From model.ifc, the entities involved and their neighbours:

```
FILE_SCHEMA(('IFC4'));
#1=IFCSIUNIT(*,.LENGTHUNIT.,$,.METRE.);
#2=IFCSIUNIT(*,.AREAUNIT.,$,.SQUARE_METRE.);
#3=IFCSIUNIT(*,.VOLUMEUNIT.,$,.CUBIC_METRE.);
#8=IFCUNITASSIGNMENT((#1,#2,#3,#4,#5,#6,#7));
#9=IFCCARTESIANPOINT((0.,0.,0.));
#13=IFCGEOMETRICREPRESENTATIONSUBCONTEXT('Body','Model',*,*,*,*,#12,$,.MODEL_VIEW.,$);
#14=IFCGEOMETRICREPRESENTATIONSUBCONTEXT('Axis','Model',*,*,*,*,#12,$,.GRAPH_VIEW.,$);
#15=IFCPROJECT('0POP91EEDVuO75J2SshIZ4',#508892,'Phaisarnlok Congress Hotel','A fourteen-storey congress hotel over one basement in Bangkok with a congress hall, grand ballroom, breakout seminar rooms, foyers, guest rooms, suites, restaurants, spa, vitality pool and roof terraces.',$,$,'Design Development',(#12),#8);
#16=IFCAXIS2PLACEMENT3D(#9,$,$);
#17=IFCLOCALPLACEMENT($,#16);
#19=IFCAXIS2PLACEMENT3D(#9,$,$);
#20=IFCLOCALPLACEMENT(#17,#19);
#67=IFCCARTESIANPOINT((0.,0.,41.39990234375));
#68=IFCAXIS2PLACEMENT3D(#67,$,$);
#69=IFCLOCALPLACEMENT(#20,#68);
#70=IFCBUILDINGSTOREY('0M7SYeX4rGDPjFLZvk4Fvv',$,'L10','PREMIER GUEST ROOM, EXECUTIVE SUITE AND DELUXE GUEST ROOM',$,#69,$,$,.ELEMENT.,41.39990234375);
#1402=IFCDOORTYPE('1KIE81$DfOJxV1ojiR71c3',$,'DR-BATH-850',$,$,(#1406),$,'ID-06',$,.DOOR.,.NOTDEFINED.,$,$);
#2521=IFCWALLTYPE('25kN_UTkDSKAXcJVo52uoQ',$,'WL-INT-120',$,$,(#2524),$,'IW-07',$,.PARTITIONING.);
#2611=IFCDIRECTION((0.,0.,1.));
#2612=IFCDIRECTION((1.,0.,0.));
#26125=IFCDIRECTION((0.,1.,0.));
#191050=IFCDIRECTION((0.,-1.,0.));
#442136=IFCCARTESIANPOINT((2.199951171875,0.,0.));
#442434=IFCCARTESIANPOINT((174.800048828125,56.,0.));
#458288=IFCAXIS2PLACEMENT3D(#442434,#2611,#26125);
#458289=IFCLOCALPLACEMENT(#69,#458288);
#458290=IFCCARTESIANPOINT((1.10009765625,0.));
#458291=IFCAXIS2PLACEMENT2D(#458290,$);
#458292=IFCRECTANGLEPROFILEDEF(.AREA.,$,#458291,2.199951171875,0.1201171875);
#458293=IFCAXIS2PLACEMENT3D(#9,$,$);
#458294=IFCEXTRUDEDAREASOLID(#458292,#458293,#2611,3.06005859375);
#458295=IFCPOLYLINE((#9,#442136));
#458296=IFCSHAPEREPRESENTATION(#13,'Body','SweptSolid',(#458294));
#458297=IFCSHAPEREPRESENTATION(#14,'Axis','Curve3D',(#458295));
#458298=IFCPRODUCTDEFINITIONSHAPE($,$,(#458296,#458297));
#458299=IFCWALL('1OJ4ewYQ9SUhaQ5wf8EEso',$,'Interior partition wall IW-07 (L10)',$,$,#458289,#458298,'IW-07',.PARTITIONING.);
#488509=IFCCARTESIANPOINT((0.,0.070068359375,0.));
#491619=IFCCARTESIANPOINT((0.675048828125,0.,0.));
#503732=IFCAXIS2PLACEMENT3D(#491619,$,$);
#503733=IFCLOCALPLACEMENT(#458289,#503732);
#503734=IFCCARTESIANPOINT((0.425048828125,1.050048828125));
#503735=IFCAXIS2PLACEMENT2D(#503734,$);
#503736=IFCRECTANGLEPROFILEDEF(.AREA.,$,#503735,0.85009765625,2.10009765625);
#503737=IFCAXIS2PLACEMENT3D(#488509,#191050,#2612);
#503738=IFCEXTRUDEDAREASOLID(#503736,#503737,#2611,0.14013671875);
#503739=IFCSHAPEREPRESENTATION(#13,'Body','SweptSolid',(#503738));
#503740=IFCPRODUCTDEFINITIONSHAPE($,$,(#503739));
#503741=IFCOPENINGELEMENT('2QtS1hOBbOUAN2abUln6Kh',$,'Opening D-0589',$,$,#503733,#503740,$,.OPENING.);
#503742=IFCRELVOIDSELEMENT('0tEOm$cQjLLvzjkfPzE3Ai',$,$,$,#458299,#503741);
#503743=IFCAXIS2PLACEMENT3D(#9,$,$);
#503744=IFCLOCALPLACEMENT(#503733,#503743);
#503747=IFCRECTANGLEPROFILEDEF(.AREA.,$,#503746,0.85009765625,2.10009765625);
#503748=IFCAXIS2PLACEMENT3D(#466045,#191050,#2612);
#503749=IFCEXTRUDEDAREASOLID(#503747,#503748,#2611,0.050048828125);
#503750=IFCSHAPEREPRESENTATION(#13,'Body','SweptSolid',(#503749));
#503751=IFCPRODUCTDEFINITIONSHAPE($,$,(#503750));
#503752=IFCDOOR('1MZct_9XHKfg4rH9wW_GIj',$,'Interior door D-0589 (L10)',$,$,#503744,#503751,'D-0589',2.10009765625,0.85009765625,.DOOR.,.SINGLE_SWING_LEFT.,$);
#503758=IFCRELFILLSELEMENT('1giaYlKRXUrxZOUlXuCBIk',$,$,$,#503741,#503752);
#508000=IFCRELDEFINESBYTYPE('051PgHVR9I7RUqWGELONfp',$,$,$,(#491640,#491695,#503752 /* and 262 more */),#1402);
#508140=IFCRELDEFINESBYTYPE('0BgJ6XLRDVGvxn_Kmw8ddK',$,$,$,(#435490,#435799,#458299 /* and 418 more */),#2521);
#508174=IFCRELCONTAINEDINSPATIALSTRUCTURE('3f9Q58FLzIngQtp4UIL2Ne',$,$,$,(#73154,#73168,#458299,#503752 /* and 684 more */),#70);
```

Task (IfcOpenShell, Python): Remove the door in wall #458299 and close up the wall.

```python
import ifcopenshell
import ifcopenshell.api.feature
import ifcopenshell.api.root
import ifcopenshell.geom
import ifcopenshell.util.shape

model = ifcopenshell.open("model.ifc")
settings = ifcopenshell.geom.settings()


def volume(element):
    """Net volume in cubic metres, openings subtracted."""
    shape = ifcopenshell.geom.create_shape(settings, element)
    return ifcopenshell.util.shape.get_volume(shape.geometry)


door = model.by_id(503752)
opening = door.FillsVoids[0].RelatingOpeningElement
wall = opening.VoidsElements[0].RelatingBuildingElement
before = volume(wall)

ifcopenshell.api.root.remove_product(model, product=door)
ifcopenshell.api.feature.remove_feature(model, feature=opening)

after = volume(wall)

print(f"wall volume {before:.3f} -> {after:.3f} m3")

model.write("model_v2.ifc")
```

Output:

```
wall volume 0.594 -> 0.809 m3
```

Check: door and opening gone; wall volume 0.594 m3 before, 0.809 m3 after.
